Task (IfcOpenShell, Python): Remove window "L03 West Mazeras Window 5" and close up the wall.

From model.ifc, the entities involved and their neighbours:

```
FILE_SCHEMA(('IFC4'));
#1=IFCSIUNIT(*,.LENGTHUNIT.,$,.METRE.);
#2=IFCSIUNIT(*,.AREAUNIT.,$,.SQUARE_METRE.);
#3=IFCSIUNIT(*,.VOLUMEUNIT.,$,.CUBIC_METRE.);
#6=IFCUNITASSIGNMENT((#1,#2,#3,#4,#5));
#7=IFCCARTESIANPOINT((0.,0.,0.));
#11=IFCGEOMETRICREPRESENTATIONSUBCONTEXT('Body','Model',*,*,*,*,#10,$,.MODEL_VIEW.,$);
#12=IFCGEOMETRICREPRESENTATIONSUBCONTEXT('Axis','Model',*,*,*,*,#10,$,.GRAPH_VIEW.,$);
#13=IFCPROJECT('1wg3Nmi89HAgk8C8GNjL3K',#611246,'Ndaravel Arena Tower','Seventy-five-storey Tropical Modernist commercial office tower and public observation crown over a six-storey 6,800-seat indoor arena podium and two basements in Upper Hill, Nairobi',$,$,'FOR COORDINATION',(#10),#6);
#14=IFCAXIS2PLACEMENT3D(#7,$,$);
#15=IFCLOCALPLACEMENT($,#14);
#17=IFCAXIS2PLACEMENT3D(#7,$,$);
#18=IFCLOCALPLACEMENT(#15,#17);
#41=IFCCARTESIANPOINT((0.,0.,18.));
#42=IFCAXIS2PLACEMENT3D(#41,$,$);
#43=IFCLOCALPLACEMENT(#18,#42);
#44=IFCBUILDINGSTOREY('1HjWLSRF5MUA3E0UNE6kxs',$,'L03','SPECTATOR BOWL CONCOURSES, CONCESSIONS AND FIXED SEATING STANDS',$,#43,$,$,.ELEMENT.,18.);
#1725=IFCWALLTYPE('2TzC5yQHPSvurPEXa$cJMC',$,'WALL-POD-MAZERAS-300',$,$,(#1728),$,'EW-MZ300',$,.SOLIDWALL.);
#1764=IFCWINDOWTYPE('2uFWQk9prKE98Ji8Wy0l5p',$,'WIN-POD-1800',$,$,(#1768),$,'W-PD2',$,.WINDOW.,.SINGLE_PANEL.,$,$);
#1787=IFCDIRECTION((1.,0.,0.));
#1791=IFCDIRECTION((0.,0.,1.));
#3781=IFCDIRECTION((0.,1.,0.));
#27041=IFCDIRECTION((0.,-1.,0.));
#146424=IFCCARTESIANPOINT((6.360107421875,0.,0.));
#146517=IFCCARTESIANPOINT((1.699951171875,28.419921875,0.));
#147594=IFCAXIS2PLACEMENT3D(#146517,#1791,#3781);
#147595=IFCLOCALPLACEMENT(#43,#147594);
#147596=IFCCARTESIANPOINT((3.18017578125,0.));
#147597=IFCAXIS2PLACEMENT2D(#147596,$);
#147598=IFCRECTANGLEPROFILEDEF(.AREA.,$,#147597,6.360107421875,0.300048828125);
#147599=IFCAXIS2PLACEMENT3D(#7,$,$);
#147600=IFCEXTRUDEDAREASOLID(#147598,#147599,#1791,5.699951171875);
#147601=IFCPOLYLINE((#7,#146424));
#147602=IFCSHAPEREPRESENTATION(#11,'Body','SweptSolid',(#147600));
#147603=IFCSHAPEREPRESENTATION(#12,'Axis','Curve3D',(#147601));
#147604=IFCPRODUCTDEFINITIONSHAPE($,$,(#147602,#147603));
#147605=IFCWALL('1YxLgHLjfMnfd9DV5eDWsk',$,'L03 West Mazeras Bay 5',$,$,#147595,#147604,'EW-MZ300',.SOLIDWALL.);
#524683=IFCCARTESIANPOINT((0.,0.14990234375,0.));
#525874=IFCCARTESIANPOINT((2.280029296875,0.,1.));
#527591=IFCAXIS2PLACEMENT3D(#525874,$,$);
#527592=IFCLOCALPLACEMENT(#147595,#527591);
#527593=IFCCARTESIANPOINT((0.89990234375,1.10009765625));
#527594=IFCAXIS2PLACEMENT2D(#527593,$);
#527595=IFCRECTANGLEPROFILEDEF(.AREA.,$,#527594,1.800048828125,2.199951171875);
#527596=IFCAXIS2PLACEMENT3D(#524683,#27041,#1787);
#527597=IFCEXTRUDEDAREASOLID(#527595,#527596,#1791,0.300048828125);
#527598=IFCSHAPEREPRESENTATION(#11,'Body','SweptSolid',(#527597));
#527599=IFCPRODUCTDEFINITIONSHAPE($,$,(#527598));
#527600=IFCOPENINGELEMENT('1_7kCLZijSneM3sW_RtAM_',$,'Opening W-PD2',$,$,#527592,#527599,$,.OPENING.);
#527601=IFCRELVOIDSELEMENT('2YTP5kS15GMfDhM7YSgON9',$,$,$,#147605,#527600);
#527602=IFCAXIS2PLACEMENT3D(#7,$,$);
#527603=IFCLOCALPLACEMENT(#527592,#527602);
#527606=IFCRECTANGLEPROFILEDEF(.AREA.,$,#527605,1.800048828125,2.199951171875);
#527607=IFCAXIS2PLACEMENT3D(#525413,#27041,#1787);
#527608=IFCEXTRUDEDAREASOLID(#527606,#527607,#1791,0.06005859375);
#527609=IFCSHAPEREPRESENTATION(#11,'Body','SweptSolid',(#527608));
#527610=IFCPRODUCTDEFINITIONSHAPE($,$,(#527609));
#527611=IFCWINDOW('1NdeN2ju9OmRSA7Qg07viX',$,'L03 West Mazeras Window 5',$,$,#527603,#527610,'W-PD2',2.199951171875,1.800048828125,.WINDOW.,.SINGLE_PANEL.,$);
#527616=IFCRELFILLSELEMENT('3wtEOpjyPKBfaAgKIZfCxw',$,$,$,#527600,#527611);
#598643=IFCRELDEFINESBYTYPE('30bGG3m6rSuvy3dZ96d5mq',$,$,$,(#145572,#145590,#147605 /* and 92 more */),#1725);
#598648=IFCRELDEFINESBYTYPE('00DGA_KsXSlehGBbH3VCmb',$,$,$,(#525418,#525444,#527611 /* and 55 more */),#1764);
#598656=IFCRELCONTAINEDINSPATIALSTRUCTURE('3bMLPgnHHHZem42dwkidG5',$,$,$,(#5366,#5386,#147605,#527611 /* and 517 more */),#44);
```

```python
import ifcopenshell
import ifcopenshell.api.feature
import ifcopenshell.api.root
import ifcopenshell.geom
import ifcopenshell.util.shape

model = ifcopenshell.open("model.ifc")
settings = ifcopenshell.geom.settings()


def volume(element):
    """Net volume in cubic metres, openings subtracted."""
    shape = ifcopenshell.geom.create_shape(settings, element)
    return ifcopenshell.util.shape.get_volume(shape.geometry)


window = model.by_id(527611)
opening = window.FillsVoids[0].RelatingOpeningElement
wall = opening.VoidsElements[0].RelatingBuildingElement
before = volume(wall)

ifcopenshell.api.root.remove_product(model, product=window)
ifcopenshell.api.feature.remove_feature(model, feature=opening)

after = volume(wall)

print(f"wall volume {before:.3f} -> {after:.3f} m3")

model.write("model-out.ifc")
```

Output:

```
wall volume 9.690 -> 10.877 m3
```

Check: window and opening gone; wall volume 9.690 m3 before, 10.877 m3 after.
